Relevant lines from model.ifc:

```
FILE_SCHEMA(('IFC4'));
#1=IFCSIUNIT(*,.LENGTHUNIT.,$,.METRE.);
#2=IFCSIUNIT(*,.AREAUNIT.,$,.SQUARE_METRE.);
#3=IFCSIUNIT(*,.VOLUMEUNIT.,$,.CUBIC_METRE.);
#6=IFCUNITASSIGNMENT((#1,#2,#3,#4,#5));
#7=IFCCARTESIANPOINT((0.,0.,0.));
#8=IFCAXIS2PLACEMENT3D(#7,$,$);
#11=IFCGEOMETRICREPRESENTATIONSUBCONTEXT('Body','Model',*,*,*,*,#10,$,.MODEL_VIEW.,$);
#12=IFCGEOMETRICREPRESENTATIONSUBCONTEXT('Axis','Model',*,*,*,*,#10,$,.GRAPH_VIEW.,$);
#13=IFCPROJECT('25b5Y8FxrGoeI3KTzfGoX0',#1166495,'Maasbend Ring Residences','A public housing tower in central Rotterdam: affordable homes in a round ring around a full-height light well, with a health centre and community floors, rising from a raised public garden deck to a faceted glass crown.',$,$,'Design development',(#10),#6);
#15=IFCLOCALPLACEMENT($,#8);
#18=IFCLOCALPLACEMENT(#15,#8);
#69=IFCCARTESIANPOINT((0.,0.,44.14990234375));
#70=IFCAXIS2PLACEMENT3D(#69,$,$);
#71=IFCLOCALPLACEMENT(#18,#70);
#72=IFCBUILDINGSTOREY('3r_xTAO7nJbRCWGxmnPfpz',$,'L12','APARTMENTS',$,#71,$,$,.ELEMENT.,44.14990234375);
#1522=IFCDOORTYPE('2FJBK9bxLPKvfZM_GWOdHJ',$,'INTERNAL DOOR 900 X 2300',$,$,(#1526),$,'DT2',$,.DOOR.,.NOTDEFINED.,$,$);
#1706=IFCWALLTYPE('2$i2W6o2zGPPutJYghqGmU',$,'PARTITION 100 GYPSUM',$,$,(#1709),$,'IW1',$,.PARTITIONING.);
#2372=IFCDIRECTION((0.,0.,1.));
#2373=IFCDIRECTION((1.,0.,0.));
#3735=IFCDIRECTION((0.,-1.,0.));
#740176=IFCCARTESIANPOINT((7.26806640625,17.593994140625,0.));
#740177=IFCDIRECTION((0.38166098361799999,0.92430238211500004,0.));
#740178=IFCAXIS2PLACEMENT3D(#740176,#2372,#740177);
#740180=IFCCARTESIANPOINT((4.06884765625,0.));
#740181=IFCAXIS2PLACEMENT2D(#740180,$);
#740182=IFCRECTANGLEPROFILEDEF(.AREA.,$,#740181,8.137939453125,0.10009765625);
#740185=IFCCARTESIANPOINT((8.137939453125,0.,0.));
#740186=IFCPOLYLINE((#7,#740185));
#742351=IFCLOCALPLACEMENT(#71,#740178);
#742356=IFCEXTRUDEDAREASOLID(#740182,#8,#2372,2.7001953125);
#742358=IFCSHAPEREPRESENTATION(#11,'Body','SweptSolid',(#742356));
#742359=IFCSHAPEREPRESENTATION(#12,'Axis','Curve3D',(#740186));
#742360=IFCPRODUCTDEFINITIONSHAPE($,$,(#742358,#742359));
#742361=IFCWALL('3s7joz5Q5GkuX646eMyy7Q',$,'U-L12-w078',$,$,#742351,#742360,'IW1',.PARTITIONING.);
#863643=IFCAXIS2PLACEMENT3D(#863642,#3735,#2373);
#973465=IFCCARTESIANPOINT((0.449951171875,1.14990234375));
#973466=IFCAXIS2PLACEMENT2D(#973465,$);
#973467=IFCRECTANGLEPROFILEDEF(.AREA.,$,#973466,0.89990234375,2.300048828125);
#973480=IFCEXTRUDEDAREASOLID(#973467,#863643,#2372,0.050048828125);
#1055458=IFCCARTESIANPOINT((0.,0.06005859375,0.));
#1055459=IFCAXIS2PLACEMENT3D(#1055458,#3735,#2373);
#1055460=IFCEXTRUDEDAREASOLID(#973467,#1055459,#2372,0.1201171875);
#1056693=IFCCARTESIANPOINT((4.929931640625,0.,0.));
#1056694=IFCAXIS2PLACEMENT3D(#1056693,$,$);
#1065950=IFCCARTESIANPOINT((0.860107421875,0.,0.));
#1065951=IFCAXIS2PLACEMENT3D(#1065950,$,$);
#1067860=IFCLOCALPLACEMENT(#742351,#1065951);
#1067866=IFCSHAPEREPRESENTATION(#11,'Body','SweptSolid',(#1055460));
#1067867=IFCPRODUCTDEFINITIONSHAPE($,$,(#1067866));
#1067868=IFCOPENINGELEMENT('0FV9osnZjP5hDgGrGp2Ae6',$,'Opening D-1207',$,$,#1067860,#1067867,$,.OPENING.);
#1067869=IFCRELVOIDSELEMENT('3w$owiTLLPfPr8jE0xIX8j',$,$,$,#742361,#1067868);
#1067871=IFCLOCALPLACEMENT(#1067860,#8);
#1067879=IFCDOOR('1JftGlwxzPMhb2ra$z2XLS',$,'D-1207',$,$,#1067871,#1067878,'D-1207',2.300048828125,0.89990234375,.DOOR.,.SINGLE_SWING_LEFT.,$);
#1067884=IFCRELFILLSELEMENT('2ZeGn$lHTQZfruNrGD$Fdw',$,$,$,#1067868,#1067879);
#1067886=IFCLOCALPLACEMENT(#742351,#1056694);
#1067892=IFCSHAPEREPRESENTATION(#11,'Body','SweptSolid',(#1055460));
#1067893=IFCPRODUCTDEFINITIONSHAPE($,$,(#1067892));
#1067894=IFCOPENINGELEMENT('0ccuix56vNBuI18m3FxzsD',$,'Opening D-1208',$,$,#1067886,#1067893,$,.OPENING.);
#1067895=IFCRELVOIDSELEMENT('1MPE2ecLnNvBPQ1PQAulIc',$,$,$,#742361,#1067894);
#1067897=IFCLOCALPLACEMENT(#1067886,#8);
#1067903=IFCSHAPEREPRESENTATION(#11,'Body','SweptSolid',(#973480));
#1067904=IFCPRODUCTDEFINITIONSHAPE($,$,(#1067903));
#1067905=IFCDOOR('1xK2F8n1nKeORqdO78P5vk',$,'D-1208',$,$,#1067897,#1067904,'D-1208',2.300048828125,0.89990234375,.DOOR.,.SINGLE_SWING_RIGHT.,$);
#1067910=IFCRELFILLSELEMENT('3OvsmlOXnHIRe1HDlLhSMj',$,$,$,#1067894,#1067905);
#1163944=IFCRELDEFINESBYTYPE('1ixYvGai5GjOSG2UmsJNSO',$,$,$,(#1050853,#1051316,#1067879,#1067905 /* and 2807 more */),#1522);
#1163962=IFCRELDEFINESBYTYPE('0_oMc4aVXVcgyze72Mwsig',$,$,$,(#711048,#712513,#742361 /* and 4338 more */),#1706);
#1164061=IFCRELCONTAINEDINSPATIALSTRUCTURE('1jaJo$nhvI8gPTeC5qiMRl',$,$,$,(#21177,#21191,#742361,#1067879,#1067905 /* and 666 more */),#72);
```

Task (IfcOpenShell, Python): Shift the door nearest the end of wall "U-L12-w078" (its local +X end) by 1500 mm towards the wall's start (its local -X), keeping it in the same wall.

```python
import ifcopenshell
import ifcopenshell.api.geometry
import ifcopenshell.util.placement
import ifcopenshell.util.unit

model = ifcopenshell.open("model.ifc")
unit_scale = ifcopenshell.util.unit.calculate_unit_scale(model)

door = model.by_guid("1xK2F8n1nKeORqdO78P5vk")
opening = door.FillsVoids[0].RelatingOpeningElement
wall = opening.VoidsElements[0].RelatingBuildingElement

wall_matrix = ifcopenshell.util.placement.get_local_placement(wall.ObjectPlacement)
shift = wall_matrix[:3, 0] * -1.5 / unit_scale
before = ifcopenshell.util.placement.get_local_placement(door.ObjectPlacement)[:3, 3].copy()

# The door is placed relative to its opening, so it follows when the opening moves.
matrix = ifcopenshell.util.placement.get_local_placement(opening.ObjectPlacement)
matrix[:3, 3] += shift
ifcopenshell.api.geometry.edit_object_placement(
    model, product=opening, matrix=matrix, is_si=False, should_transform_children=True
)

after = ifcopenshell.util.placement.get_local_placement(door.ObjectPlacement)[:3, 3]
print("door moved by", (after - before).round(3) + 0.0)

model.write("model-out.ifc")
```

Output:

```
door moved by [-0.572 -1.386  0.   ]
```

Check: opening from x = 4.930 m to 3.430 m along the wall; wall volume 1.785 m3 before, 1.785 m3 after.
